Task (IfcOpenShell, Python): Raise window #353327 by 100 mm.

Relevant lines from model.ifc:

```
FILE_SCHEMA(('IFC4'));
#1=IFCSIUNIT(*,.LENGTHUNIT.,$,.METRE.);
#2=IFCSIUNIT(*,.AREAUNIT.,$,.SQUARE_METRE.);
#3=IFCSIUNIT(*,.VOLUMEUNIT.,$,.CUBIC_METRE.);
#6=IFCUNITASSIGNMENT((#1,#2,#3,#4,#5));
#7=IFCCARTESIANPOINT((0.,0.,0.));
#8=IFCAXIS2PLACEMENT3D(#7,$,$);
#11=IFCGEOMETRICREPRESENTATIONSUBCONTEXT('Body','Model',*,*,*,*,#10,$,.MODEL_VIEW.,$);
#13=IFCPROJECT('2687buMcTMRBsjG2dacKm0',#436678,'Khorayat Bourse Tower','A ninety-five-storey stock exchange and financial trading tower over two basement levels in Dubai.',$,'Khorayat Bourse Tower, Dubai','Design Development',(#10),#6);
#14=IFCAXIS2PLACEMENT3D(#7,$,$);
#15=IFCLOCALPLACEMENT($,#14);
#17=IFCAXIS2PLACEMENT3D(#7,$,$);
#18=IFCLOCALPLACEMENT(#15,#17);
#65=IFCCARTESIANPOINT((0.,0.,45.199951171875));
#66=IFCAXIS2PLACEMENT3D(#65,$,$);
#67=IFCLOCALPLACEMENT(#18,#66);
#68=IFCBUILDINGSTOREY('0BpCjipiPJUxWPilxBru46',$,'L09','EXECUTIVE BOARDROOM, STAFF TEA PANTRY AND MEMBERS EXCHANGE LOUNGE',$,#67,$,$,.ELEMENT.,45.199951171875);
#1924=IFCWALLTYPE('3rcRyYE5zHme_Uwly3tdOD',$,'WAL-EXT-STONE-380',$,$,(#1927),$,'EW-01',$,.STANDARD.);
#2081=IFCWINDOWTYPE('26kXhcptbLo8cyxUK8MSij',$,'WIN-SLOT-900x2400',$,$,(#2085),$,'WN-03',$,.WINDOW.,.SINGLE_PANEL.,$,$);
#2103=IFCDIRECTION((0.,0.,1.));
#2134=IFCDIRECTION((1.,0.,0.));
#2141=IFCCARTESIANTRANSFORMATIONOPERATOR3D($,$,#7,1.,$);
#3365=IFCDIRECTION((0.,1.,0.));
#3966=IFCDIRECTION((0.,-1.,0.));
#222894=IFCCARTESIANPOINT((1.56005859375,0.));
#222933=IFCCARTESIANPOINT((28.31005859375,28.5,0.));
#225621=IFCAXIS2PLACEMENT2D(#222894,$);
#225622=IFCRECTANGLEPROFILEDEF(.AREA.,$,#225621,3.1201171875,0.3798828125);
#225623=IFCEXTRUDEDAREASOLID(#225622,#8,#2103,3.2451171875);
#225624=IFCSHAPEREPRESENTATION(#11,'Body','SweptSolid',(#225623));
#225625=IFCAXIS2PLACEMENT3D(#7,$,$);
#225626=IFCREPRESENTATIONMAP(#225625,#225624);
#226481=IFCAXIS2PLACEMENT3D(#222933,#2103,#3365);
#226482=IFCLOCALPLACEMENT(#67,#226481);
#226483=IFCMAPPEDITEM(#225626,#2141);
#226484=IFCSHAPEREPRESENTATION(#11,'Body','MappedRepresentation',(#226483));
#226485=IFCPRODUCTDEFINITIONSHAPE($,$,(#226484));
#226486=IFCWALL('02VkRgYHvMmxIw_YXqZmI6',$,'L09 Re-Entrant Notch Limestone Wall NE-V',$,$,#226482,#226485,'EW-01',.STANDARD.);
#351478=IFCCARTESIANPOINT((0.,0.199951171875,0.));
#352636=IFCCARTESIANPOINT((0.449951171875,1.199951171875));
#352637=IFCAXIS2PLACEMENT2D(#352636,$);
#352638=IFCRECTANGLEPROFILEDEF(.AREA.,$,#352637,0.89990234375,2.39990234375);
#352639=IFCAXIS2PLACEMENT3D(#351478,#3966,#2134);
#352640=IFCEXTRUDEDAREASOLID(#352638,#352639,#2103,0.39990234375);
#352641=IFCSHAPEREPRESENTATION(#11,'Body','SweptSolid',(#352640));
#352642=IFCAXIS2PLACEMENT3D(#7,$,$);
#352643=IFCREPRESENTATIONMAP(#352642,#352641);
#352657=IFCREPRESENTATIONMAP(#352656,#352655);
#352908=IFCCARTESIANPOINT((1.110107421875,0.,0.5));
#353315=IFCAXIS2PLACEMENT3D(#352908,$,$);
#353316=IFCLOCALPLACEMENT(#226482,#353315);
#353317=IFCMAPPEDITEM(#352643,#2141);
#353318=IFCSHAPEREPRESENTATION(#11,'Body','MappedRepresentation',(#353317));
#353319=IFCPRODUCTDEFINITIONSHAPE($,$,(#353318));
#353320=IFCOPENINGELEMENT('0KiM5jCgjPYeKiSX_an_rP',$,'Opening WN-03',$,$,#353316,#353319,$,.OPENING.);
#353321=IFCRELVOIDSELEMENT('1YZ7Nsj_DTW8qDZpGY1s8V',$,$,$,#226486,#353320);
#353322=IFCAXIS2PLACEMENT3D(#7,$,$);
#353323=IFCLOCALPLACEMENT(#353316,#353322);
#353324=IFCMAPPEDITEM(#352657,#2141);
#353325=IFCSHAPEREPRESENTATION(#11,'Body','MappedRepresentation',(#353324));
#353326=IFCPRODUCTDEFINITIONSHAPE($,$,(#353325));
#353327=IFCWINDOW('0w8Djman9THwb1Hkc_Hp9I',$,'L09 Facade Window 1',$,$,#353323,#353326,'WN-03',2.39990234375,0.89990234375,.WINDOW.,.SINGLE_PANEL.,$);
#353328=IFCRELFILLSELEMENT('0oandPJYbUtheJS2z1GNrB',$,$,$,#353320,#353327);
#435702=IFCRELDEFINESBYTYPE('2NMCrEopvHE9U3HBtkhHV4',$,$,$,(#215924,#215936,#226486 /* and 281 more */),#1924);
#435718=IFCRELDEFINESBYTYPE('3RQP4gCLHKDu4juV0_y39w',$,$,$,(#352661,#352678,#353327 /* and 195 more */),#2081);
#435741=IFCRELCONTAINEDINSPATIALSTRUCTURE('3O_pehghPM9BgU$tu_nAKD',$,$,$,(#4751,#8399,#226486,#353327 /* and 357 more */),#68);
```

```python
import numpy as np
import ifcopenshell
import ifcopenshell.api.geometry
import ifcopenshell.util.placement
import ifcopenshell.util.unit

model = ifcopenshell.open("model.ifc")
unit_scale = ifcopenshell.util.unit.calculate_unit_scale(model)

window = model.by_guid("0w8Djman9THwb1Hkc_Hp9I")
opening = window.FillsVoids[0].RelatingOpeningElement
dz = 0.1

shift = np.array([0.0, 0.0, dz])
# The window is placed relative to its opening, so it follows when the opening moves.
matrix = ifcopenshell.util.placement.get_local_placement(opening.ObjectPlacement)
matrix[:3, 3] += shift
ifcopenshell.api.geometry.edit_object_placement(
    model, product=opening, matrix=matrix, is_si=False, should_transform_children=True
)

print(f"moved by {dz * unit_scale:+.3f} m")

model.write("model_v2.ifc")
```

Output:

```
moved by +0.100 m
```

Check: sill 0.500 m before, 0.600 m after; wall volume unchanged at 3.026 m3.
